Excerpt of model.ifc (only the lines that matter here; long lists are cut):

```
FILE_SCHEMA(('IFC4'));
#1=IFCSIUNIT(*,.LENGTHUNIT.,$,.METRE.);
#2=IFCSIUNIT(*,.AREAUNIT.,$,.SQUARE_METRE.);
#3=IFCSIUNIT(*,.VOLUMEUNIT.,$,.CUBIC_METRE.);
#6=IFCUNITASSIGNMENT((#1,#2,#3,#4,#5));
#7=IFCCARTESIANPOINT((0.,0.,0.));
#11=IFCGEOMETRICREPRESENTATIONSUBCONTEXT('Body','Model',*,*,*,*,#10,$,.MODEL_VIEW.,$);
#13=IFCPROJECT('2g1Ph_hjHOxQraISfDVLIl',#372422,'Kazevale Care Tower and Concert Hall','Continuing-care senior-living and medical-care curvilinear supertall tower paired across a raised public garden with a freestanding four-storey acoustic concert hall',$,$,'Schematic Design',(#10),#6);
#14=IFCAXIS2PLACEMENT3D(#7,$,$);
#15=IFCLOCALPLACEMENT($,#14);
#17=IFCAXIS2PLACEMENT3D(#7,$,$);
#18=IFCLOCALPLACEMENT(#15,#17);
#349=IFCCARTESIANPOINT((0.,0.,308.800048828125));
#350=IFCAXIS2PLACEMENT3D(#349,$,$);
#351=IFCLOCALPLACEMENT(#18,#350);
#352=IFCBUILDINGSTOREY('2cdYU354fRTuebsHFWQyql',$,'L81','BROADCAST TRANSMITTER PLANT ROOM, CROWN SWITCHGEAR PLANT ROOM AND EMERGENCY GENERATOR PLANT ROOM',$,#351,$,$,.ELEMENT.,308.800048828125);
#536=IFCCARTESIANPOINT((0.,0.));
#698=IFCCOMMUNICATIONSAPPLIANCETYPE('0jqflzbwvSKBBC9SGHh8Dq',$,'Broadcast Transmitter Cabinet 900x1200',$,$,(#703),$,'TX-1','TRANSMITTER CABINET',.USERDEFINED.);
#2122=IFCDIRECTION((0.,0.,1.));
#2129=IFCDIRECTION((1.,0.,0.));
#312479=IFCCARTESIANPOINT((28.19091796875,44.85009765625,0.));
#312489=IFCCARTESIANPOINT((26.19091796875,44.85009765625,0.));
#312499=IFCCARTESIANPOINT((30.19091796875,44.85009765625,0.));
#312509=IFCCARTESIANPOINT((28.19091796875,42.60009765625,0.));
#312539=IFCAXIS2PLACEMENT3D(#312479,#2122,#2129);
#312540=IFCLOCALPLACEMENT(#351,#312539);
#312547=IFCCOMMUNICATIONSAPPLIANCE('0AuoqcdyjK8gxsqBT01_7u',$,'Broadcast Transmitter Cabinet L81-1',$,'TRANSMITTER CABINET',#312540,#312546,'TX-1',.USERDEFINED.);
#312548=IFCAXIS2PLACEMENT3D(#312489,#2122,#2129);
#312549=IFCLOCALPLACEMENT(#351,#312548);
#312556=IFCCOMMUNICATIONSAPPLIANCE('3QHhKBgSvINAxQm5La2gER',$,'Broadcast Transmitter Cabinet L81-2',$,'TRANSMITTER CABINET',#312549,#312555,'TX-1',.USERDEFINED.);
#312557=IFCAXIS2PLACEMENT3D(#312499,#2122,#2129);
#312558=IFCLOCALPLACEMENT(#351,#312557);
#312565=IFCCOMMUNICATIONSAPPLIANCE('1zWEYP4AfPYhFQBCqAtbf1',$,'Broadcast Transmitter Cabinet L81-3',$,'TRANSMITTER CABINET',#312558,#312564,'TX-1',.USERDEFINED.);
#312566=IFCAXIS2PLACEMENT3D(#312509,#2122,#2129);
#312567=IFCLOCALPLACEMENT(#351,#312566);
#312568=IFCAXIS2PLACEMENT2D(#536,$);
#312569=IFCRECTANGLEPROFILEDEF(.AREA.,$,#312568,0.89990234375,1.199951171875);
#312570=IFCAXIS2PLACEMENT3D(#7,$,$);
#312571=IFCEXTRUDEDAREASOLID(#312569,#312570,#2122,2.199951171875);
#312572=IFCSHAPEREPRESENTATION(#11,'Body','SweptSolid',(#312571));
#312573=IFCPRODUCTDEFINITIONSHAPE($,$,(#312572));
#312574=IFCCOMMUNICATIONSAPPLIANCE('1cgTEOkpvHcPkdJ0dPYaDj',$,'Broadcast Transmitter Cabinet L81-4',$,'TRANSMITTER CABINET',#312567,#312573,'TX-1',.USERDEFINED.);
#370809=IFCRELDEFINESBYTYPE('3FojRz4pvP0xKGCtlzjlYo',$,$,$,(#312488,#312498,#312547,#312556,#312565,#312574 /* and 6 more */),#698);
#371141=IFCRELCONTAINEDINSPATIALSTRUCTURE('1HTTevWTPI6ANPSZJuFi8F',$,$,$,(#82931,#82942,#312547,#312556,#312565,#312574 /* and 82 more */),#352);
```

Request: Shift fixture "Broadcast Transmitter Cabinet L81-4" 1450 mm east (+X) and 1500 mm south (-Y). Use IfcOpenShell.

```python
import ifcopenshell
import ifcopenshell.api.geometry
import ifcopenshell.util.placement
import ifcopenshell.util.unit

model = ifcopenshell.open("model.ifc")
unit_scale = ifcopenshell.util.unit.calculate_unit_scale(model)

item = model.by_guid("1cgTEOkpvHcPkdJ0dPYaDj")
matrix = ifcopenshell.util.placement.get_local_placement(item.ObjectPlacement)
matrix[0, 3] += 1.45 / unit_scale
matrix[1, 3] -= 1.5 / unit_scale
ifcopenshell.api.geometry.edit_object_placement(model, product=item, matrix=matrix, is_si=False)

print(ifcopenshell.util.placement.get_local_placement(item.ObjectPlacement).round(3) + 0.0)

model.write("model_updated.ifc")
```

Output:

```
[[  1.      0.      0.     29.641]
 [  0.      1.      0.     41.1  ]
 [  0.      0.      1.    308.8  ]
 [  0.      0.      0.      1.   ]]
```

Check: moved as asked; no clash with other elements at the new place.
